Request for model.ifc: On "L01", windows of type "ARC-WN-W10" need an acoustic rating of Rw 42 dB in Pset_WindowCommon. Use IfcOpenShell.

First a look at what the model holds.

```python
import ifcopenshell
import ifcopenshell.util.element

model = ifcopenshell.open("model.ifc")
print(model.schema)
storey = next(s for s in model.by_type("IfcBuildingStorey") if s.Name == "L01")
windows = [e for e in ifcopenshell.util.element.get_decomposition(storey) if e.is_a("IfcWindow")]
seen = {}
for e in windows:
    element_type = ifcopenshell.util.element.get_type(e)
    key = (element_type.Name if element_type != e and element_type else None, ifcopenshell.util.element.get_pset(e, "Pset_WindowCommon", "AcousticRating"))
    seen[key] = seen.get(key, 0) + 1
for (name, value), count in sorted(seen.items(), key=str):
    print(count, "x", name, "|", value)
```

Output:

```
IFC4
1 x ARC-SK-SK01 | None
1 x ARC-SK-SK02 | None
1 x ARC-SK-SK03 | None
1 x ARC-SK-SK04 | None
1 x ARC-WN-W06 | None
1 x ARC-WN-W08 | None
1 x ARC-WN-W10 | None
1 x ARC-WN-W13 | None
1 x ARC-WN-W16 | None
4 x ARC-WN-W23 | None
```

```python
import ifcopenshell
import ifcopenshell.api.pset
import ifcopenshell.util.element

model = ifcopenshell.open("model.ifc")

storey = next(s for s in model.by_type("IfcBuildingStorey") if s.Name == "L01")
windows = [e for e in ifcopenshell.util.element.get_decomposition(storey) if e.is_a("IfcWindow")]

count = 0
for e in windows:
    element_type = ifcopenshell.util.element.get_type(e)
    if element_type in (None, e) or element_type.Name != "ARC-WN-W10":
        continue
    # add_pset returns the element's existing set when there is one.
    pset = ifcopenshell.api.pset.add_pset(model, product=e, name="Pset_WindowCommon")
    ifcopenshell.api.pset.edit_pset(model, pset=pset, properties={"AcousticRating": "Rw 42 dB"})
    count += 1

print(count, "windows updated")

model.write("model_rev.ifc")
```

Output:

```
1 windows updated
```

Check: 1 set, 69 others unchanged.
